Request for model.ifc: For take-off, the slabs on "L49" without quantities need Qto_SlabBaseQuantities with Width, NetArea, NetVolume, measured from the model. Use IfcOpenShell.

First a look at what the model holds.

```python
import ifcopenshell
import ifcopenshell.util.element
import ifcopenshell.util.unit

model = ifcopenshell.open("model.ifc")
print(model.schema)
for unit_type in ("LENGTHUNIT", "AREAUNIT", "VOLUMEUNIT"):
    print(unit_type, ifcopenshell.util.unit.calculate_unit_scale(model, unit_type))
storey = next(s for s in model.by_type("IfcBuildingStorey") if s.Name == "L49")
slabs = [e for e in ifcopenshell.util.element.get_decomposition(storey) if e.is_a("IfcSlab")]
for e in sorted(slabs, key=lambda e: e.id()):
    print(e.id(), e.is_a(), e.Name, list(ifcopenshell.util.element.get_psets(e, qtos_only=True)), sep=" | ")
```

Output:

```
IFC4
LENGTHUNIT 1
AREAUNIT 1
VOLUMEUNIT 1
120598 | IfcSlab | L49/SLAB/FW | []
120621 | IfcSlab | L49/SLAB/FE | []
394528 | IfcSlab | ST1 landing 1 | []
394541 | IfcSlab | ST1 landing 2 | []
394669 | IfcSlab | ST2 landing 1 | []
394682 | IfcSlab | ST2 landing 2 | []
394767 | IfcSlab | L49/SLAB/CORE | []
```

```python
import ifcopenshell
import ifcopenshell.api.pset
import ifcopenshell.geom
import ifcopenshell.util.element
import ifcopenshell.util.shape
import ifcopenshell.util.unit

model = ifcopenshell.open("model.ifc")
unit_scale = ifcopenshell.util.unit.calculate_unit_scale(model)
area_scale = ifcopenshell.util.unit.calculate_unit_scale(model, "AREAUNIT")
volume_scale = ifcopenshell.util.unit.calculate_unit_scale(model, "VOLUMEUNIT")
settings = ifcopenshell.geom.settings()

storey = next(s for s in model.by_type("IfcBuildingStorey") if s.Name == "L49")
slabs = [e for e in ifcopenshell.util.element.get_decomposition(storey) if e.is_a("IfcSlab")]

for e in sorted(slabs, key=lambda e: e.id()):
    if ifcopenshell.util.element.get_psets(e, qtos_only=True, should_inherit=False):
        continue
    # Geometry comes back in metres, in the element's own axes.
    shape = ifcopenshell.geom.create_shape(settings, e)
    values = {
        "Width": ifcopenshell.util.shape.get_z(shape.geometry) / unit_scale,
        "NetArea": ifcopenshell.util.shape.get_footprint_area(shape.geometry) / area_scale,
        "NetVolume": ifcopenshell.util.shape.get_volume(shape.geometry) / volume_scale,
    }
    qto = ifcopenshell.api.pset.add_qto(model, product=e, name="Qto_SlabBaseQuantities")
    ifcopenshell.api.pset.edit_qto(model, qto=qto, properties=values)
    print(e.id(), {k: round(v, 3) for k, v in values.items()})

model.write("model_v2.ifc")
```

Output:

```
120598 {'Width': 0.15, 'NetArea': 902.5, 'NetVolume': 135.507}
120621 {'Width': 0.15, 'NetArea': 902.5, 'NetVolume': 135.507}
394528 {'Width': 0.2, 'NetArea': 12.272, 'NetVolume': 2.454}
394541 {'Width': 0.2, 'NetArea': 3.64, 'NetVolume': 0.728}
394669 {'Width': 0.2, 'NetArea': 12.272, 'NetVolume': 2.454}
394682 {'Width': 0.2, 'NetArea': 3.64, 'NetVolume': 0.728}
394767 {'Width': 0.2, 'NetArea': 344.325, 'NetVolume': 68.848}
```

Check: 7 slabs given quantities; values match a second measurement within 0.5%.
